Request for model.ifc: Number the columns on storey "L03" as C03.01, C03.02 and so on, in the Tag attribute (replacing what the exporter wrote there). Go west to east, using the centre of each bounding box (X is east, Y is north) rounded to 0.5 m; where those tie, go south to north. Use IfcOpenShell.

First a look at what the model holds.

```python
import ifcopenshell
import ifcopenshell.util.element
import ifcopenshell.util.placement

model = ifcopenshell.open("model.ifc")
print(model.schema)
storey = next(s for s in model.by_type("IfcBuildingStorey") if s.Name == "L03")
columns = [e for e in ifcopenshell.util.element.get_decomposition(storey) if e.is_a("IfcColumn")]
for e in sorted(columns, key=lambda e: e.id()):
    origin = ifcopenshell.util.placement.get_local_placement(e.ObjectPlacement)[:3, 3]
    print(e.id(), e.Tag, e.Name, origin.round(2) + 0.0, sep=" | ")
```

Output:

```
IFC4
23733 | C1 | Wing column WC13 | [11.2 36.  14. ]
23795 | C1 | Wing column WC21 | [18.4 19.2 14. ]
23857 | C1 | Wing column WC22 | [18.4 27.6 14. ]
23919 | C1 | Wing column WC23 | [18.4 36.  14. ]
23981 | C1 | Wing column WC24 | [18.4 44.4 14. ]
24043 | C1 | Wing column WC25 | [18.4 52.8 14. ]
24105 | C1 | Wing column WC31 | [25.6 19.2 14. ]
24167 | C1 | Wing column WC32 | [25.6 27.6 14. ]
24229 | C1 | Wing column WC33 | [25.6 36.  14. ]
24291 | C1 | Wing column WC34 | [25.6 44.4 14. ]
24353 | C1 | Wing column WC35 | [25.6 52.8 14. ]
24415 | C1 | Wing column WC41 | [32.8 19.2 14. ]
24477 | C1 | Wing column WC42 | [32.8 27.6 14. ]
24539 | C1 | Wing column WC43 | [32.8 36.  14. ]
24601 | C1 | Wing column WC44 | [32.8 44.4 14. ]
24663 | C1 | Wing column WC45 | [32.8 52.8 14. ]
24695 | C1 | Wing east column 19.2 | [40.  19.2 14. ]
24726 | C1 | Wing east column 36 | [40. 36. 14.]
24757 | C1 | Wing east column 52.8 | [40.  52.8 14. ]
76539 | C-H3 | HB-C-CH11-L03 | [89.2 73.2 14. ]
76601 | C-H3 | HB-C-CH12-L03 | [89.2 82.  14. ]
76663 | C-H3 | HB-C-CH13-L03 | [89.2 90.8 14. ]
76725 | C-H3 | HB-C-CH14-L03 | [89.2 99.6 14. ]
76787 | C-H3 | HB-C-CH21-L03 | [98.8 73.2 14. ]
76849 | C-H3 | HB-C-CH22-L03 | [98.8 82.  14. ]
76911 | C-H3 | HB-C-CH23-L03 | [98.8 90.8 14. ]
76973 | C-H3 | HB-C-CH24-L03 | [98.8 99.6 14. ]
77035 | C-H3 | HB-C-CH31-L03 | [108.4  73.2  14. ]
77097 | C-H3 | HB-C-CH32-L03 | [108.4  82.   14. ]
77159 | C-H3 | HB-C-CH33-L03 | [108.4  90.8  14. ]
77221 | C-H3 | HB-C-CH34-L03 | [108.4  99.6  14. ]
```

```python
import ifcopenshell
import ifcopenshell.geom
import ifcopenshell.util.element
import ifcopenshell.util.shape

model = ifcopenshell.open("model.ifc")
settings = ifcopenshell.geom.settings()
settings.set("use-world-coords", True)


def centre(element):
    shape = ifcopenshell.geom.create_shape(settings, element)
    return ifcopenshell.util.shape.get_bbox_centroid(shape.geometry)


storey = next(s for s in model.by_type("IfcBuildingStorey") if s.Name == "L03")
columns = [e for e in ifcopenshell.util.element.get_decomposition(storey) if e.is_a("IfcColumn")]

# Insertion points can sit at a corner or the storey origin, so sort by the geometry (in metres).
centres = {e: centre(e) for e in columns}
columns.sort(key=lambda e: (round(centres[e][0] / 0.5), centres[e][1]))

for i, e in enumerate(columns, start=1):
    number = f"C03.{i:02d}"
    e.Tag = number
    print(e.id(), number)

model.write("model_edited.ifc")
```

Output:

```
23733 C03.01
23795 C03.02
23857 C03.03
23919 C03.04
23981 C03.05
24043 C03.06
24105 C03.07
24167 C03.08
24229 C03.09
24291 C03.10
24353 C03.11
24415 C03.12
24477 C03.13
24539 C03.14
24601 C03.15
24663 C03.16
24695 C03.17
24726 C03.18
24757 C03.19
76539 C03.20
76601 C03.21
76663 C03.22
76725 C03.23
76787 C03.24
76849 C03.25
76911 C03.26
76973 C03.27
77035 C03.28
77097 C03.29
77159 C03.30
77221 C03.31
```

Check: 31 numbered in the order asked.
